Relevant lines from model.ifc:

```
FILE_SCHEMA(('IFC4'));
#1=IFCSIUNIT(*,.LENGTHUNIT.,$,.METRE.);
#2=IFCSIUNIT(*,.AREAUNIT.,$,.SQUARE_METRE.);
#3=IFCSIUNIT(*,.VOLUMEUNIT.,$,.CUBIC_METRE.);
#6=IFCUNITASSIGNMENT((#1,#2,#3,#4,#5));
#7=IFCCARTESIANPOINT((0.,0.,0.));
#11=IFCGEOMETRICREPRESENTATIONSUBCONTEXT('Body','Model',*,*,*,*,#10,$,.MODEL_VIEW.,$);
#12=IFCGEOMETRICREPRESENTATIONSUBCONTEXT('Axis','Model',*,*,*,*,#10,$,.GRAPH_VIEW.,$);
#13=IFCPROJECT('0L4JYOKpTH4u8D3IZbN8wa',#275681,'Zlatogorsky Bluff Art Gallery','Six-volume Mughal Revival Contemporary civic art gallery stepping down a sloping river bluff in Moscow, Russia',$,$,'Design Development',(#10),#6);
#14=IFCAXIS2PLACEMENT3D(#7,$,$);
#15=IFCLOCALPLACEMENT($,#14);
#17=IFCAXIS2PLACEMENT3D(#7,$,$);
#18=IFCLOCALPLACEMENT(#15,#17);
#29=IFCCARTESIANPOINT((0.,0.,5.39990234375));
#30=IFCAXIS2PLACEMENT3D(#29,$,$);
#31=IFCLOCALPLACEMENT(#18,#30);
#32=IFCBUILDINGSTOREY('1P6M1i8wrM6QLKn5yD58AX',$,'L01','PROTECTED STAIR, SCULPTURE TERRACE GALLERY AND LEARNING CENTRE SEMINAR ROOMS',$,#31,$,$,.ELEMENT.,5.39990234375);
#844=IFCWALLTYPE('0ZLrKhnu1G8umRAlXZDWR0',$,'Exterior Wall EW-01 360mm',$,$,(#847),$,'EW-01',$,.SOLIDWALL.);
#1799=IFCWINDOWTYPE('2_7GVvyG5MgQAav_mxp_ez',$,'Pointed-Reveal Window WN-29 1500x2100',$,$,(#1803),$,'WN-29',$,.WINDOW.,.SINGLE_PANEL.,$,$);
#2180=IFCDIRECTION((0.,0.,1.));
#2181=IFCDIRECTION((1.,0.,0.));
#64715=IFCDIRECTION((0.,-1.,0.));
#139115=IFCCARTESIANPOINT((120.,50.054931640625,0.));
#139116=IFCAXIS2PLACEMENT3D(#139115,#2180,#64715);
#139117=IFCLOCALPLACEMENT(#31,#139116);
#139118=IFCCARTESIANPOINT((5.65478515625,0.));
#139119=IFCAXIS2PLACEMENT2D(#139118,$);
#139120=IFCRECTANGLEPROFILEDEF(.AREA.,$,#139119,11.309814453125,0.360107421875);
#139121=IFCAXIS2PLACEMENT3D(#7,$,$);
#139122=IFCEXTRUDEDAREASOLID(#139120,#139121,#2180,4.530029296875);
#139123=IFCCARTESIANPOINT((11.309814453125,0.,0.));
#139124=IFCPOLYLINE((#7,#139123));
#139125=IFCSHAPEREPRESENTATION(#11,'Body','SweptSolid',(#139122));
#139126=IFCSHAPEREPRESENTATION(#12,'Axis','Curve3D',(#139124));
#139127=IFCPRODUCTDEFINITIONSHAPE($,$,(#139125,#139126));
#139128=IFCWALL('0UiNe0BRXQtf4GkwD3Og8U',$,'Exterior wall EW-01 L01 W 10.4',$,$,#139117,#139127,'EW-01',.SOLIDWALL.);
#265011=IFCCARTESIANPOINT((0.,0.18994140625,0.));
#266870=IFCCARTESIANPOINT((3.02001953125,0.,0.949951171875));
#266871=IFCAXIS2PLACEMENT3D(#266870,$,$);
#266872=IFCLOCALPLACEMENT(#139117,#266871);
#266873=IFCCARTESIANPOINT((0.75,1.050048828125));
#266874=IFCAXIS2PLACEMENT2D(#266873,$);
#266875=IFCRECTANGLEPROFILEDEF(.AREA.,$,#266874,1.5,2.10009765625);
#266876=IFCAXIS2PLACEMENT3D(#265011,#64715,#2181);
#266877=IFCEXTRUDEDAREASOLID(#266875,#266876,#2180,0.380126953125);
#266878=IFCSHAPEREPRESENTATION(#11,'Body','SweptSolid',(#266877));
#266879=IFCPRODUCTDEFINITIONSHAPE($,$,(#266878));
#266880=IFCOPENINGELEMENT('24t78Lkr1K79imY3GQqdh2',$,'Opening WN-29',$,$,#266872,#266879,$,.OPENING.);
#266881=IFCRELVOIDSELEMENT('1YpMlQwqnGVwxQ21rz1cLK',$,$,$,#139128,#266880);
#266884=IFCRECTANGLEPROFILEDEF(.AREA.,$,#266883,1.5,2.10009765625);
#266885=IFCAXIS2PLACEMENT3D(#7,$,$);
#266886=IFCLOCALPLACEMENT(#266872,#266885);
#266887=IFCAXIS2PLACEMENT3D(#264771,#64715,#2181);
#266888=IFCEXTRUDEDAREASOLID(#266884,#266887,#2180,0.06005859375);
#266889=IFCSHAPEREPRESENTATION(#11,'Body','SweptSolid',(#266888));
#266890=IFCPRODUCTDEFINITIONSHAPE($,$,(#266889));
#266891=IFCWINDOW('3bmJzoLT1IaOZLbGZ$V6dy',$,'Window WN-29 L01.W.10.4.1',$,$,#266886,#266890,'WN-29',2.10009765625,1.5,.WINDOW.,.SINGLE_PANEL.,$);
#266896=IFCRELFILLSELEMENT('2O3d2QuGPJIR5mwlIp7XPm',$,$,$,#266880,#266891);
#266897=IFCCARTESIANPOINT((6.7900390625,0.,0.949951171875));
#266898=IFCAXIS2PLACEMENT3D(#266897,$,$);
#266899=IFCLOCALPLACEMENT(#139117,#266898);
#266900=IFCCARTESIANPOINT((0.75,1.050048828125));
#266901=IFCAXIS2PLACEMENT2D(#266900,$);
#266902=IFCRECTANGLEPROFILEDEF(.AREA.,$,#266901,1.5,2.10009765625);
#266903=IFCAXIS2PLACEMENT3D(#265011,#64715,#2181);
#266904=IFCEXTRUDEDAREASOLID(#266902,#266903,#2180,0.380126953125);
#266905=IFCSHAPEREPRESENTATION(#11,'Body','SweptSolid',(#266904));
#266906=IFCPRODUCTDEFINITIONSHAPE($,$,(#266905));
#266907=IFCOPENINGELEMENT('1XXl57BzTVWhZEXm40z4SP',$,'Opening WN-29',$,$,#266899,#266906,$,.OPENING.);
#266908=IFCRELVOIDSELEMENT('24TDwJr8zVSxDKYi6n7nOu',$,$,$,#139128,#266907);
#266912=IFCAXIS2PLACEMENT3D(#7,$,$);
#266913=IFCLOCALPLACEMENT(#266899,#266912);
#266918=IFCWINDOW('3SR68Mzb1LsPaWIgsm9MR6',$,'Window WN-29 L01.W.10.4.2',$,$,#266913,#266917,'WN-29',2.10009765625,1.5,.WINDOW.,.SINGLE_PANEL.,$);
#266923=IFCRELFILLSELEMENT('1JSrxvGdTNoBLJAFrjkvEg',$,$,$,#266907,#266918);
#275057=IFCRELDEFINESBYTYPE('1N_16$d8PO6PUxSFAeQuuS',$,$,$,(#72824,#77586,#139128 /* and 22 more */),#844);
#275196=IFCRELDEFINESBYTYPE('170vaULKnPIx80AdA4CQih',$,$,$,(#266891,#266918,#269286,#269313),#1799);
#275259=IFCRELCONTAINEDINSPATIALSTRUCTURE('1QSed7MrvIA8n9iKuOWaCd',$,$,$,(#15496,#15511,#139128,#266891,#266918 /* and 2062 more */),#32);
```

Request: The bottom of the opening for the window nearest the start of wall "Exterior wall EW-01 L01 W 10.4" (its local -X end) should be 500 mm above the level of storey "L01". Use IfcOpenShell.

```python
import numpy as np
import ifcopenshell
import ifcopenshell.api.geometry
import ifcopenshell.geom
import ifcopenshell.util.element
import ifcopenshell.util.placement
import ifcopenshell.util.shape
import ifcopenshell.util.unit

model = ifcopenshell.open("model.ifc")
unit_scale = ifcopenshell.util.unit.calculate_unit_scale(model)

window = model.by_guid("3bmJzoLT1IaOZLbGZ$V6dy")
opening = window.FillsVoids[0].RelatingOpeningElement
storey = ifcopenshell.util.element.get_container(window, ifc_class="IfcBuildingStorey")
level = ifcopenshell.util.placement.get_local_placement(storey.ObjectPlacement)[2, 3]

# The opening's origin need not be at the sill, so measure its lowest point.
shape = ifcopenshell.geom.create_shape(ifcopenshell.geom.settings(), opening)
bottom = ifcopenshell.util.shape.get_shape_bottom_elevation(shape, shape.geometry) / unit_scale
dz = level + 0.5 / unit_scale - bottom

shift = np.array([0.0, 0.0, dz])
# The window is placed relative to its opening, so it follows when the opening moves.
matrix = ifcopenshell.util.placement.get_local_placement(opening.ObjectPlacement)
matrix[:3, 3] += shift
ifcopenshell.api.geometry.edit_object_placement(
    model, product=opening, matrix=matrix, is_si=False, should_transform_children=True
)

print(f"moved by {dz * unit_scale:+.3f} m")

model.write("model_edited.ifc")
```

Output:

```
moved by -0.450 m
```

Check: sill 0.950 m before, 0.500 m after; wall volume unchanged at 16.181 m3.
